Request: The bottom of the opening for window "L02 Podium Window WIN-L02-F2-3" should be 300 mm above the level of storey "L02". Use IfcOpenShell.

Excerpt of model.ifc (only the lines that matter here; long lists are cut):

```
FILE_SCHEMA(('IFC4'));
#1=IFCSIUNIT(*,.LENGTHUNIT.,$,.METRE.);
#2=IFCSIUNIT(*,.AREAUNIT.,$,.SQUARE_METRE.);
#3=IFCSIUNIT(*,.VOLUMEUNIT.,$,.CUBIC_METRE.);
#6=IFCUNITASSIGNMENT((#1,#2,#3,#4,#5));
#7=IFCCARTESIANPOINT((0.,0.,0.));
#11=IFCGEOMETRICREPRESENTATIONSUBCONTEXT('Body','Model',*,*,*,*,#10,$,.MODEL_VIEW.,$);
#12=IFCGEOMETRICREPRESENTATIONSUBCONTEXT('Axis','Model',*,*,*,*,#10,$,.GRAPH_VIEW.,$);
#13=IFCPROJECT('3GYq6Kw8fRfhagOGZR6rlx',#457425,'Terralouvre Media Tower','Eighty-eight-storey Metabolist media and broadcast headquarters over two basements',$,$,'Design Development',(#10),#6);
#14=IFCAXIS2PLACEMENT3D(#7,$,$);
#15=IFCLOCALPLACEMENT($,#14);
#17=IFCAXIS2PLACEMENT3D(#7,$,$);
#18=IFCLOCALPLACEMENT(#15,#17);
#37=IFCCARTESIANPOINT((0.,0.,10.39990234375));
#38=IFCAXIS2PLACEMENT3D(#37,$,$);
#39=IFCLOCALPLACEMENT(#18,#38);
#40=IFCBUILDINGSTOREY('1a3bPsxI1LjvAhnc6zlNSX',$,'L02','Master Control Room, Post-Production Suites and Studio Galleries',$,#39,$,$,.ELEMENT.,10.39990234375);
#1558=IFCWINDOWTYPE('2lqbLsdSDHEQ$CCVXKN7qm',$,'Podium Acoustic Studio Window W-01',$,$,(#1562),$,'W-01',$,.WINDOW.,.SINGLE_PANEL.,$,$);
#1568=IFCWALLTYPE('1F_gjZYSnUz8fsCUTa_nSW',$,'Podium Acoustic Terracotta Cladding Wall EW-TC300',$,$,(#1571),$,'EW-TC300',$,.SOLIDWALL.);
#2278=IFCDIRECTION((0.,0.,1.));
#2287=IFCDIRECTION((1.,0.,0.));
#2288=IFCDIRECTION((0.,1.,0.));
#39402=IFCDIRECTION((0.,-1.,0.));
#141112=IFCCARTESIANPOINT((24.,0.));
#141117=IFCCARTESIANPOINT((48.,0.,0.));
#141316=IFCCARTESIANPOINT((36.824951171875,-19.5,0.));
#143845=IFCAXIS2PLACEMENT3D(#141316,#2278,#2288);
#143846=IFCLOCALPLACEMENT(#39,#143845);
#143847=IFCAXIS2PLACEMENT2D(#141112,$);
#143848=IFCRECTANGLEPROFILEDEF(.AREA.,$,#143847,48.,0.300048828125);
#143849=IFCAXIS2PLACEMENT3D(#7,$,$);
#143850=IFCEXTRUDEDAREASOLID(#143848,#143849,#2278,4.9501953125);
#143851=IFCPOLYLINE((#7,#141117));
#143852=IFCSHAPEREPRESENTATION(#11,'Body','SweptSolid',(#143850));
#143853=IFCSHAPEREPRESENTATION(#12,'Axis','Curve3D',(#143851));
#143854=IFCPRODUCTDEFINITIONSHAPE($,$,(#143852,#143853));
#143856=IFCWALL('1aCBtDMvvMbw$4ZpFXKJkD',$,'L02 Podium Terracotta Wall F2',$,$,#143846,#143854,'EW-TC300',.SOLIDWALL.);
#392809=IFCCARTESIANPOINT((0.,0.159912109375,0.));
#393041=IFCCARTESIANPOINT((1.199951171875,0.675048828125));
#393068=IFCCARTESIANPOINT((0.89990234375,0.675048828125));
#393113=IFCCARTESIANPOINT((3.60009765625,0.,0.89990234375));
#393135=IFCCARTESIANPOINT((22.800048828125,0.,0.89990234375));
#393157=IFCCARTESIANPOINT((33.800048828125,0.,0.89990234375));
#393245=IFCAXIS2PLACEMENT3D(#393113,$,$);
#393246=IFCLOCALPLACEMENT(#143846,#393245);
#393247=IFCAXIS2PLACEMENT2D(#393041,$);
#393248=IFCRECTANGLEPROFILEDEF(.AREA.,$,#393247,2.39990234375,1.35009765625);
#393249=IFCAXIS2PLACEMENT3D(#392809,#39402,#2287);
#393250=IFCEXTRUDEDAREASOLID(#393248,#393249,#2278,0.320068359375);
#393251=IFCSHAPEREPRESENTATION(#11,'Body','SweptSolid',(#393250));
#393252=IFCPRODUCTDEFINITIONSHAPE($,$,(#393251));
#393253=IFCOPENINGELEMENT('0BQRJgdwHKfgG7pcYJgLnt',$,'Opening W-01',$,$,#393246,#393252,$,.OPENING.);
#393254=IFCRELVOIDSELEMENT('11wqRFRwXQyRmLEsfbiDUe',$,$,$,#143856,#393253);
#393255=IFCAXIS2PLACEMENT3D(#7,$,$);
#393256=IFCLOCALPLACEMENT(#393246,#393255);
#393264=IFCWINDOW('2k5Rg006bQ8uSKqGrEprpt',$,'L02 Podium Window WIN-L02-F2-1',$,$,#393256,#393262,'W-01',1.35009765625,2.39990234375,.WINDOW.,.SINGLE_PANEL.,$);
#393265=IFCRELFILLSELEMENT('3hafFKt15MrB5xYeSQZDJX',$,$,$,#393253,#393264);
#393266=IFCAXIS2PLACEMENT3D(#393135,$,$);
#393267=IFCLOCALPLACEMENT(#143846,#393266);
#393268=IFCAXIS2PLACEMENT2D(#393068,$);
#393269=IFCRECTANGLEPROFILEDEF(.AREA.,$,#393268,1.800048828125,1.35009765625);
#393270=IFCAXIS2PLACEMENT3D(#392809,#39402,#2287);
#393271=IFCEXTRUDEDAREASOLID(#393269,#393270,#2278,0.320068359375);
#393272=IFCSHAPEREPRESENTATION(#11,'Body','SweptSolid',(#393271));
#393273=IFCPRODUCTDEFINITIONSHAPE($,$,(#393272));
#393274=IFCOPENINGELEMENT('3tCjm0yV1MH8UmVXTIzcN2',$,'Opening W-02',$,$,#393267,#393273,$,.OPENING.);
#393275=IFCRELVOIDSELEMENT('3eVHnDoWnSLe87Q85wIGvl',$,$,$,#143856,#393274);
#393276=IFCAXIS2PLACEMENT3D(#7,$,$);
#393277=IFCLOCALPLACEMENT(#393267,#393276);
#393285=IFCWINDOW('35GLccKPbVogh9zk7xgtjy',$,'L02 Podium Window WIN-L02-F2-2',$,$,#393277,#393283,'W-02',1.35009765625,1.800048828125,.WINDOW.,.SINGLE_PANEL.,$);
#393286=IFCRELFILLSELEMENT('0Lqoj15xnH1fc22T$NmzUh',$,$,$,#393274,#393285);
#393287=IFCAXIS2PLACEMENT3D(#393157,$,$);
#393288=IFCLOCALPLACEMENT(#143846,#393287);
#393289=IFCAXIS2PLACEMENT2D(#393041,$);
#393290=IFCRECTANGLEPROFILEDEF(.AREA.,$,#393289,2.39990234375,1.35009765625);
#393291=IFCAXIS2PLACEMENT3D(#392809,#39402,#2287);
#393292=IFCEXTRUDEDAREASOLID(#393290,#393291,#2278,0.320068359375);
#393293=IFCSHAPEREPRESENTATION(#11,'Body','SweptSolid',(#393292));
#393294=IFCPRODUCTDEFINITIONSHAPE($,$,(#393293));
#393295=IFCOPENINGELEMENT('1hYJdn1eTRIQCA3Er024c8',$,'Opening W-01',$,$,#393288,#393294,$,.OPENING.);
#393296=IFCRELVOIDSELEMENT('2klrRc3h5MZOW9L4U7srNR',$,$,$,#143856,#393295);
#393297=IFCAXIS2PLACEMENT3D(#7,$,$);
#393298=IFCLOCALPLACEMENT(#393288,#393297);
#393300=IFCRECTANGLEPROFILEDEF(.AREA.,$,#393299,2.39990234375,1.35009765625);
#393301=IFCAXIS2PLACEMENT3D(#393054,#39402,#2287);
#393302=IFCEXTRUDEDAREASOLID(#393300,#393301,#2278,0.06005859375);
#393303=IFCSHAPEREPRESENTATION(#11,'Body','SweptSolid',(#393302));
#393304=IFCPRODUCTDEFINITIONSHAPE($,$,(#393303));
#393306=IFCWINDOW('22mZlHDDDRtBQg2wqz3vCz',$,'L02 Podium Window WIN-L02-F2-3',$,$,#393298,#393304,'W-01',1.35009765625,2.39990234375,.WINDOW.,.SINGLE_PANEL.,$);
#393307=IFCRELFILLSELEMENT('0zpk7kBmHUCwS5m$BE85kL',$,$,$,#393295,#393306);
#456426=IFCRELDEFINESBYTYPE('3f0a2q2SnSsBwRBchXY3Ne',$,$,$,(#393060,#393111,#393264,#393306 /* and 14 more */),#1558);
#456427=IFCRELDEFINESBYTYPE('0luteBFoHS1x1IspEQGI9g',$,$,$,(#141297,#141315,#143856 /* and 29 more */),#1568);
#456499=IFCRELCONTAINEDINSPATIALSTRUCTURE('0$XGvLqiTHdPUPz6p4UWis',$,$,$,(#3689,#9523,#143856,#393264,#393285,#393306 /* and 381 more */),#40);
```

```python
import numpy as np
import ifcopenshell
import ifcopenshell.api.geometry
import ifcopenshell.geom
import ifcopenshell.util.element
import ifcopenshell.util.placement
import ifcopenshell.util.shape
import ifcopenshell.util.unit

model = ifcopenshell.open("model.ifc")
unit_scale = ifcopenshell.util.unit.calculate_unit_scale(model)

window = model.by_guid("22mZlHDDDRtBQg2wqz3vCz")
opening = window.FillsVoids[0].RelatingOpeningElement
storey = ifcopenshell.util.element.get_container(window, ifc_class="IfcBuildingStorey")
level = ifcopenshell.util.placement.get_local_placement(storey.ObjectPlacement)[2, 3]

# The opening's origin need not be at the sill, so measure its lowest point.
shape = ifcopenshell.geom.create_shape(ifcopenshell.geom.settings(), opening)
bottom = ifcopenshell.util.shape.get_shape_bottom_elevation(shape, shape.geometry) / unit_scale
dz = level + 0.3 / unit_scale - bottom

shift = np.array([0.0, 0.0, dz])
# The window is placed relative to its opening, so it follows when the opening moves.
matrix = ifcopenshell.util.placement.get_local_placement(opening.ObjectPlacement)
matrix[:3, 3] += shift
ifcopenshell.api.geometry.edit_object_placement(
    model, product=opening, matrix=matrix, is_si=False, should_transform_children=True
)

print(f"moved by {dz * unit_scale:+.3f} m")

model.write("model_v2.ifc")
```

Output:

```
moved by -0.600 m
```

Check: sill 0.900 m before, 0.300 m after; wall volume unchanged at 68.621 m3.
